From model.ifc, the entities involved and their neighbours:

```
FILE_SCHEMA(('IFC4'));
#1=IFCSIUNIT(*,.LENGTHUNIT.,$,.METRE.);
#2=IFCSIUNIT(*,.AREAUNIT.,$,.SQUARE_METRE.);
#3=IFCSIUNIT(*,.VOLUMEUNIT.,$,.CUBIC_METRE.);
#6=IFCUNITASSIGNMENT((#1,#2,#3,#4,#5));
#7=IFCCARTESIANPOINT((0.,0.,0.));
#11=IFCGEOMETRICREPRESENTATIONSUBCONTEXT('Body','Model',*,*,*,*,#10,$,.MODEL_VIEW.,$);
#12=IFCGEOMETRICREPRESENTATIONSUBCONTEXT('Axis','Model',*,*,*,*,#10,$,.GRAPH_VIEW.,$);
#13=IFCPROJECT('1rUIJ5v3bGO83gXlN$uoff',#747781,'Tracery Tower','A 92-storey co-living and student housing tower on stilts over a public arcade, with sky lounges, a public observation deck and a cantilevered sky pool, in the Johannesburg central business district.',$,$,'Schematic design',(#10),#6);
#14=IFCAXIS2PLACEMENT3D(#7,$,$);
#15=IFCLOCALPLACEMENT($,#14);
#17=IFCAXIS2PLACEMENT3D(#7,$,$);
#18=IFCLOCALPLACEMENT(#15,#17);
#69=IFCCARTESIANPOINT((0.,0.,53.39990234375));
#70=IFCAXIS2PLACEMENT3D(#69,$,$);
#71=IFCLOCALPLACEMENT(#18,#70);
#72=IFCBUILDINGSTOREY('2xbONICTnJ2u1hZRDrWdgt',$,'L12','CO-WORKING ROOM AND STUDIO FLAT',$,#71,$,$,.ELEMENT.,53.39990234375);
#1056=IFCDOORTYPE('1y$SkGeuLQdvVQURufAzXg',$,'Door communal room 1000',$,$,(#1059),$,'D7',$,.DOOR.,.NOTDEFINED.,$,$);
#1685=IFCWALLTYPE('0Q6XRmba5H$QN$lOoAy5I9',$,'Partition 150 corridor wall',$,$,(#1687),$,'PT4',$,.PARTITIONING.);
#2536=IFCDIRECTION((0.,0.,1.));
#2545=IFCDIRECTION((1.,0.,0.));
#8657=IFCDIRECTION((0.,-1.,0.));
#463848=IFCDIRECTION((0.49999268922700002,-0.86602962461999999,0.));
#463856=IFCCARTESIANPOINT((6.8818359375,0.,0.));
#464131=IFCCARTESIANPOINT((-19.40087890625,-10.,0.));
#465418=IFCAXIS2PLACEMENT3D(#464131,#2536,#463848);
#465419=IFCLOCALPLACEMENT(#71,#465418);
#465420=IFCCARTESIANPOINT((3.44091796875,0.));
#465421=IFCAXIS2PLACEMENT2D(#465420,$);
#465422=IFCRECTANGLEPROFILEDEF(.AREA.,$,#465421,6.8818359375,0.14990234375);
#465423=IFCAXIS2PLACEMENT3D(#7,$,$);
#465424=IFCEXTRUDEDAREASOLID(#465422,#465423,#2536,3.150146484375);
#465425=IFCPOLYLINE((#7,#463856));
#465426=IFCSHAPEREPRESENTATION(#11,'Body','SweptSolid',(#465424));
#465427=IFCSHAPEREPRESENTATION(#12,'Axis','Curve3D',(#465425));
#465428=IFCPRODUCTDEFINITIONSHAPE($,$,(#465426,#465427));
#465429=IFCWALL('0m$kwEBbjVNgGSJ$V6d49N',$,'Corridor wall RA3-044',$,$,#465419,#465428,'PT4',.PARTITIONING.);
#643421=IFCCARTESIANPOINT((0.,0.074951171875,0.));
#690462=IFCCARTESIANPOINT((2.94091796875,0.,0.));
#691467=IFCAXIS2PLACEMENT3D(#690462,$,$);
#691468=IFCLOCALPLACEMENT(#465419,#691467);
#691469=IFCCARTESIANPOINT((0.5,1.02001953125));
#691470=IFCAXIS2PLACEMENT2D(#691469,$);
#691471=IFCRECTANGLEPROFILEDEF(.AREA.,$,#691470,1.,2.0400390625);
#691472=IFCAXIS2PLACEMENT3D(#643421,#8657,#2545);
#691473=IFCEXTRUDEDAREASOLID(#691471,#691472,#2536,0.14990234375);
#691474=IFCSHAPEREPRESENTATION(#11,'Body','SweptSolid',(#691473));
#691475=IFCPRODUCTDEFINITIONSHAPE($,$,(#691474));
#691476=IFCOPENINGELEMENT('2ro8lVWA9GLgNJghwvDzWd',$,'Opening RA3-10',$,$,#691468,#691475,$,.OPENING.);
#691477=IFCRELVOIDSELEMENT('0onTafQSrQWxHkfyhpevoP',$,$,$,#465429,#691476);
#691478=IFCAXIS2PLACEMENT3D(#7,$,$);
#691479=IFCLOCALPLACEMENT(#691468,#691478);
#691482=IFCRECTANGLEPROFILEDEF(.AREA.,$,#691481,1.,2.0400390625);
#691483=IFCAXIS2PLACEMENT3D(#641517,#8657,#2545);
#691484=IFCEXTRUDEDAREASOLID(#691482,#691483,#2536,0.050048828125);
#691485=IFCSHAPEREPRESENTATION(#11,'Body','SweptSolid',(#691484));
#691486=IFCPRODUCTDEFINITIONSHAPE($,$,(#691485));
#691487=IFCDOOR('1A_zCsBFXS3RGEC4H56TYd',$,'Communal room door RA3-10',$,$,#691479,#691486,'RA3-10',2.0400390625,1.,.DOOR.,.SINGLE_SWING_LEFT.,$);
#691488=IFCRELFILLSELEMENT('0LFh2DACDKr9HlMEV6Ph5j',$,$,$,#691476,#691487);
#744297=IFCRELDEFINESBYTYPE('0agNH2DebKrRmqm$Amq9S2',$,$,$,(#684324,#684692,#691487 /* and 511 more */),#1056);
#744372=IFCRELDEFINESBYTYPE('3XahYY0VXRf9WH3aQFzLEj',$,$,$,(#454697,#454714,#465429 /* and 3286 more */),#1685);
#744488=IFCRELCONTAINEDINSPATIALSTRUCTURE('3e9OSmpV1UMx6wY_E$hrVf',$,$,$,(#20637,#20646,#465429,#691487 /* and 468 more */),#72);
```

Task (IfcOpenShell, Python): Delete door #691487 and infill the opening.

```python
import ifcopenshell
import ifcopenshell.api.feature
import ifcopenshell.api.root
import ifcopenshell.geom
import ifcopenshell.util.shape

model = ifcopenshell.open("model.ifc")
settings = ifcopenshell.geom.settings()


def volume(element):
    """Net volume in cubic metres, openings subtracted."""
    shape = ifcopenshell.geom.create_shape(settings, element)
    return ifcopenshell.util.shape.get_volume(shape.geometry)


door = model.by_guid("1A_zCsBFXS3RGEC4H56TYd")
opening = door.FillsVoids[0].RelatingOpeningElement
wall = opening.VoidsElements[0].RelatingBuildingElement
before = volume(wall)

ifcopenshell.api.root.remove_product(model, product=door)
ifcopenshell.api.feature.remove_feature(model, feature=opening)

after = volume(wall)

print(f"wall volume {before:.3f} -> {after:.3f} m3")

model.write("model_updated.ifc")
```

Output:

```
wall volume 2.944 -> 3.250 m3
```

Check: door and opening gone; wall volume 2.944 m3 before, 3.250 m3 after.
